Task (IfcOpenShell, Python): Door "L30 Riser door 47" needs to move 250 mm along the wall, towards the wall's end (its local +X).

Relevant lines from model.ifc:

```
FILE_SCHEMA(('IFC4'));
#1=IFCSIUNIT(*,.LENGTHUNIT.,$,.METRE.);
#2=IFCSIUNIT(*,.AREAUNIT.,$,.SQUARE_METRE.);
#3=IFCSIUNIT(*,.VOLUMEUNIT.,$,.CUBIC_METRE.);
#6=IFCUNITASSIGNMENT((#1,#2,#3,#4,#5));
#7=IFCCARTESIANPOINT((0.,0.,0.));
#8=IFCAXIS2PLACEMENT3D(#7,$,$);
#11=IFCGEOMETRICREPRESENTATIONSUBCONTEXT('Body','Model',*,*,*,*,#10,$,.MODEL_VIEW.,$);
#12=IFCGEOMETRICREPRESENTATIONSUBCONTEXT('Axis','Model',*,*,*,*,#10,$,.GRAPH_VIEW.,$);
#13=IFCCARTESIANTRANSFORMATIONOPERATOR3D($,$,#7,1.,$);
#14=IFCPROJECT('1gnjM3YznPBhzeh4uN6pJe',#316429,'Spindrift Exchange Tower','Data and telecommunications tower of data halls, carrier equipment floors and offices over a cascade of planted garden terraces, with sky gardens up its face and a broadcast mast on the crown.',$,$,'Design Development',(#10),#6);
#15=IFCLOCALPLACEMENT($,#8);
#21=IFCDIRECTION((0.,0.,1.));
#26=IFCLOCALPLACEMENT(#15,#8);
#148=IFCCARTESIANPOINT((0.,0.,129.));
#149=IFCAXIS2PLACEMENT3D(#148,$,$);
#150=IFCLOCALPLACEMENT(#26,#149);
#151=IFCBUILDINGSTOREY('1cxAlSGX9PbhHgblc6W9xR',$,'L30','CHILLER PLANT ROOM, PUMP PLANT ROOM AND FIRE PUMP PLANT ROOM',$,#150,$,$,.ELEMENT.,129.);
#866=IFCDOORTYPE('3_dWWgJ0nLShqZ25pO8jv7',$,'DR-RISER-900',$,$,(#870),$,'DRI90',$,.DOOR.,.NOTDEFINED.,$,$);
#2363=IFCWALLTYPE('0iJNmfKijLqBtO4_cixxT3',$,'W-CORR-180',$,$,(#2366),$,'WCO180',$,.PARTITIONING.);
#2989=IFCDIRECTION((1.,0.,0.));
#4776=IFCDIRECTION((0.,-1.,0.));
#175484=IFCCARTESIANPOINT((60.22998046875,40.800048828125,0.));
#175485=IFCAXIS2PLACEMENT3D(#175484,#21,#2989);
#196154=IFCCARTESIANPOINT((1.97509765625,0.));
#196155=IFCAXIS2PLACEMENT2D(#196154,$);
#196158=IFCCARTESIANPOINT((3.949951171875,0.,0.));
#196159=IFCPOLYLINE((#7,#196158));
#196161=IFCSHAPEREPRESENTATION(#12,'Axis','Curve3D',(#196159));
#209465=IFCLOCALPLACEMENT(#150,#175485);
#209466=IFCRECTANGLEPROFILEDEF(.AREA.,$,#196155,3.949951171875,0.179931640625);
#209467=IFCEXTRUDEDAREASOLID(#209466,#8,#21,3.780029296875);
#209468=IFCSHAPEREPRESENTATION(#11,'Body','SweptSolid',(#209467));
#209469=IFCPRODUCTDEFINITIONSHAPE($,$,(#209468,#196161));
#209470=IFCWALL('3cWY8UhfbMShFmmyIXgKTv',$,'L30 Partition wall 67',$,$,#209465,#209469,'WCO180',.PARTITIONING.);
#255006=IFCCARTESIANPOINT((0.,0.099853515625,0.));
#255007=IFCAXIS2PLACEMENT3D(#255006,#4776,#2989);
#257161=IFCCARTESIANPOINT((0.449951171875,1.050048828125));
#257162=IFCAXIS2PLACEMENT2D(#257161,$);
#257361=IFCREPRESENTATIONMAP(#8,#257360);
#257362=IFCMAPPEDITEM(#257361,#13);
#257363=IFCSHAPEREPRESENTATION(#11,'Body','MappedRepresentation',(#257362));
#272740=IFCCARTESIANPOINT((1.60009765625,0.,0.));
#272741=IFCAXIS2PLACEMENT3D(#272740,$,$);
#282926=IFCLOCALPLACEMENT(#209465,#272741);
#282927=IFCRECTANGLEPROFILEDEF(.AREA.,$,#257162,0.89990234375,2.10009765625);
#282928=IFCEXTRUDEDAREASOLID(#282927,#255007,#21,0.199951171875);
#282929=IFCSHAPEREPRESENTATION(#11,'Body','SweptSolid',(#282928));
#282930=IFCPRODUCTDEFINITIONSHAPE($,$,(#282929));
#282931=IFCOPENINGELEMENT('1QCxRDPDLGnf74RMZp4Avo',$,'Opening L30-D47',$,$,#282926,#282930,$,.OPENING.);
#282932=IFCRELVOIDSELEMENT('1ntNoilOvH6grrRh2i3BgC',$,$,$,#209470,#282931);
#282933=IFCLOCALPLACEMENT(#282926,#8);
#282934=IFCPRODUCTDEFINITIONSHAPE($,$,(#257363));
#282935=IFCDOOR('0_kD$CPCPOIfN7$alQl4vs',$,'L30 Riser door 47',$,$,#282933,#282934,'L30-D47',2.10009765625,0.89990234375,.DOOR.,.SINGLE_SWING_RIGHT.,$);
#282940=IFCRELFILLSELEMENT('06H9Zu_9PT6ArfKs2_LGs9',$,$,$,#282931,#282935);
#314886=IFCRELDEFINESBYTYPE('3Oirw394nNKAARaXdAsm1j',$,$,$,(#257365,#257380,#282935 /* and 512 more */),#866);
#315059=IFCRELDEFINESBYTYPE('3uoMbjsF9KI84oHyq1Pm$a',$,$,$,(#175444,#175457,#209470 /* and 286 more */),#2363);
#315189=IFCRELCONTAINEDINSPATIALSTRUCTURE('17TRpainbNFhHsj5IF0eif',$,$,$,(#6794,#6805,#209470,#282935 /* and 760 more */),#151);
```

```python
import ifcopenshell
import ifcopenshell.api.geometry
import ifcopenshell.util.placement
import ifcopenshell.util.unit

model = ifcopenshell.open("model.ifc")
unit_scale = ifcopenshell.util.unit.calculate_unit_scale(model)

door = model.by_id(282935)
opening = door.FillsVoids[0].RelatingOpeningElement
wall = opening.VoidsElements[0].RelatingBuildingElement

wall_matrix = ifcopenshell.util.placement.get_local_placement(wall.ObjectPlacement)
shift = wall_matrix[:3, 0] * 0.25 / unit_scale
before = ifcopenshell.util.placement.get_local_placement(door.ObjectPlacement)[:3, 3].copy()

# The door is placed relative to its opening, so it follows when the opening moves.
matrix = ifcopenshell.util.placement.get_local_placement(opening.ObjectPlacement)
matrix[:3, 3] += shift
ifcopenshell.api.geometry.edit_object_placement(
    model, product=opening, matrix=matrix, is_si=False, should_transform_children=True
)

after = ifcopenshell.util.placement.get_local_placement(door.ObjectPlacement)[:3, 3]
print("door moved by", (after - before).round(3) + 0.0)

model.write("model_rev.ifc")
```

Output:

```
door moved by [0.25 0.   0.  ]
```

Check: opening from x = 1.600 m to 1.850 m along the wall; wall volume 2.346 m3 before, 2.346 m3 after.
